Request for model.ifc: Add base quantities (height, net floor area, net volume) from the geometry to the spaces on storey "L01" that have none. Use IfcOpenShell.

First a look at what the model holds.

```python
import ifcopenshell
import ifcopenshell.util.element
import ifcopenshell.util.unit

model = ifcopenshell.open("model.ifc")
print(model.schema)
for unit_type in ("LENGTHUNIT", "AREAUNIT", "VOLUMEUNIT"):
    print(unit_type, ifcopenshell.util.unit.calculate_unit_scale(model, unit_type))
storey = next(s for s in model.by_type("IfcBuildingStorey") if s.Name == "L01")
spaces = [e for e in ifcopenshell.util.element.get_decomposition(storey) if e.is_a("IfcSpace")]
for e in sorted(spaces, key=lambda e: e.id()):
    print(e.id(), e.is_a(), e.Name, list(ifcopenshell.util.element.get_psets(e, qtos_only=True)), sep=" | ")
```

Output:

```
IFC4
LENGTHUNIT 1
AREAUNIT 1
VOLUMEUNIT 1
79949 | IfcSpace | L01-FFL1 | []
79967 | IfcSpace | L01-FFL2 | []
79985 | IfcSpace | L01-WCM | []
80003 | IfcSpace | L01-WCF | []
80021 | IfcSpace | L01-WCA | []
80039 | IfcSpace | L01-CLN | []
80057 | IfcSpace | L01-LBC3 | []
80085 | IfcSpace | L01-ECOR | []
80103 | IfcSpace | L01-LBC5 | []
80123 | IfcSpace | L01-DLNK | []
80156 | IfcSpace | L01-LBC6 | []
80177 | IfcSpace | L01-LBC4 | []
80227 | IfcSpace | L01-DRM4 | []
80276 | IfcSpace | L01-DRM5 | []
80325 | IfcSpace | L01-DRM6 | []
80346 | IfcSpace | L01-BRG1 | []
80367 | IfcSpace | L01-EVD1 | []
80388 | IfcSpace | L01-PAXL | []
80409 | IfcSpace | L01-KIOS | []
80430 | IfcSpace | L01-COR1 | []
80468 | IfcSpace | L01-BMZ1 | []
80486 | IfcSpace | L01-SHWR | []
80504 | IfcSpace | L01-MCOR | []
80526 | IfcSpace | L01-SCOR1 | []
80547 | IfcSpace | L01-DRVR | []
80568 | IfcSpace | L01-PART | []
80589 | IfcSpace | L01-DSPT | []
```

```python
import ifcopenshell
import ifcopenshell.api.pset
import ifcopenshell.geom
import ifcopenshell.util.element
import ifcopenshell.util.shape
import ifcopenshell.util.unit

model = ifcopenshell.open("model.ifc")
unit_scale = ifcopenshell.util.unit.calculate_unit_scale(model)
area_scale = ifcopenshell.util.unit.calculate_unit_scale(model, "AREAUNIT")
volume_scale = ifcopenshell.util.unit.calculate_unit_scale(model, "VOLUMEUNIT")
settings = ifcopenshell.geom.settings()

storey = next(s for s in model.by_type("IfcBuildingStorey") if s.Name == "L01")
spaces = [e for e in ifcopenshell.util.element.get_decomposition(storey) if e.is_a("IfcSpace")]

for e in sorted(spaces, key=lambda e: e.id()):
    if ifcopenshell.util.element.get_psets(e, qtos_only=True, should_inherit=False):
        continue
    # Geometry comes back in metres, in the element's own axes.
    shape = ifcopenshell.geom.create_shape(settings, e)
    values = {
        "Height": ifcopenshell.util.shape.get_z(shape.geometry) / unit_scale,
        "NetFloorArea": ifcopenshell.util.shape.get_footprint_area(shape.geometry) / area_scale,
        "NetVolume": ifcopenshell.util.shape.get_volume(shape.geometry) / volume_scale,
    }
    qto = ifcopenshell.api.pset.add_qto(model, product=e, name="Qto_SpaceBaseQuantities")
    ifcopenshell.api.pset.edit_qto(model, qto=qto, properties=values)
    print(e.id(), {k: round(v, 3) for k, v in values.items()})

model.write("model_v2.ifc")
```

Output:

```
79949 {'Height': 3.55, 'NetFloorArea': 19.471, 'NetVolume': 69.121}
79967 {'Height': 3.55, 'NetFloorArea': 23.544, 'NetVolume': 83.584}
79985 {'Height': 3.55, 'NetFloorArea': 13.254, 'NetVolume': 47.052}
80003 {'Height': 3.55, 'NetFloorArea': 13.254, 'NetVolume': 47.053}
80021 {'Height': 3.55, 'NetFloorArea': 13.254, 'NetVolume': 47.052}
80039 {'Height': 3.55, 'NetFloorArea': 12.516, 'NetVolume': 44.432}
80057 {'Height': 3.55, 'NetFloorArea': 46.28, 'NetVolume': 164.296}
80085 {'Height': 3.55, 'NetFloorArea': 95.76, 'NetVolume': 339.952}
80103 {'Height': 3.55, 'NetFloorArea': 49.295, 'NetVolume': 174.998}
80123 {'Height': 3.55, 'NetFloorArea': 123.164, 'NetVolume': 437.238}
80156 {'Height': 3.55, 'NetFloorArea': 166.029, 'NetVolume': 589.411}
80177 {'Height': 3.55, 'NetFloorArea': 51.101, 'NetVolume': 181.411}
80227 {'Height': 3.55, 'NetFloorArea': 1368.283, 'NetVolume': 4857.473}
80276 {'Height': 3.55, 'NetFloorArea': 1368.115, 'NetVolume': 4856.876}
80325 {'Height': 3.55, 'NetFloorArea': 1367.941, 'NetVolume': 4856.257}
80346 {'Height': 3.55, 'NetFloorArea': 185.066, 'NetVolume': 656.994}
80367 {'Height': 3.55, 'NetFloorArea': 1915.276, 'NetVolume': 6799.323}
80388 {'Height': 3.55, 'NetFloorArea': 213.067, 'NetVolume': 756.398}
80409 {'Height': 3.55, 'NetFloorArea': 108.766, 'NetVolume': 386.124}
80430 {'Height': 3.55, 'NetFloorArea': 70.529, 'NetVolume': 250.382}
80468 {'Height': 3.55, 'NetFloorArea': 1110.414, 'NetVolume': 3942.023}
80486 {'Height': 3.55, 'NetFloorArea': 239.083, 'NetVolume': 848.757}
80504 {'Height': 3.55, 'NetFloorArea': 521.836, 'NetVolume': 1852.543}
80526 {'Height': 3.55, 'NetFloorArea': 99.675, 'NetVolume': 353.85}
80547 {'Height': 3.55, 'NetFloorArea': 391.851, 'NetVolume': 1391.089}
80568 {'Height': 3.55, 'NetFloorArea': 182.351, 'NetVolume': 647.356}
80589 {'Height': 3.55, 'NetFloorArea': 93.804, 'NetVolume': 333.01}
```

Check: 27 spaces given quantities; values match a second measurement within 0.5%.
